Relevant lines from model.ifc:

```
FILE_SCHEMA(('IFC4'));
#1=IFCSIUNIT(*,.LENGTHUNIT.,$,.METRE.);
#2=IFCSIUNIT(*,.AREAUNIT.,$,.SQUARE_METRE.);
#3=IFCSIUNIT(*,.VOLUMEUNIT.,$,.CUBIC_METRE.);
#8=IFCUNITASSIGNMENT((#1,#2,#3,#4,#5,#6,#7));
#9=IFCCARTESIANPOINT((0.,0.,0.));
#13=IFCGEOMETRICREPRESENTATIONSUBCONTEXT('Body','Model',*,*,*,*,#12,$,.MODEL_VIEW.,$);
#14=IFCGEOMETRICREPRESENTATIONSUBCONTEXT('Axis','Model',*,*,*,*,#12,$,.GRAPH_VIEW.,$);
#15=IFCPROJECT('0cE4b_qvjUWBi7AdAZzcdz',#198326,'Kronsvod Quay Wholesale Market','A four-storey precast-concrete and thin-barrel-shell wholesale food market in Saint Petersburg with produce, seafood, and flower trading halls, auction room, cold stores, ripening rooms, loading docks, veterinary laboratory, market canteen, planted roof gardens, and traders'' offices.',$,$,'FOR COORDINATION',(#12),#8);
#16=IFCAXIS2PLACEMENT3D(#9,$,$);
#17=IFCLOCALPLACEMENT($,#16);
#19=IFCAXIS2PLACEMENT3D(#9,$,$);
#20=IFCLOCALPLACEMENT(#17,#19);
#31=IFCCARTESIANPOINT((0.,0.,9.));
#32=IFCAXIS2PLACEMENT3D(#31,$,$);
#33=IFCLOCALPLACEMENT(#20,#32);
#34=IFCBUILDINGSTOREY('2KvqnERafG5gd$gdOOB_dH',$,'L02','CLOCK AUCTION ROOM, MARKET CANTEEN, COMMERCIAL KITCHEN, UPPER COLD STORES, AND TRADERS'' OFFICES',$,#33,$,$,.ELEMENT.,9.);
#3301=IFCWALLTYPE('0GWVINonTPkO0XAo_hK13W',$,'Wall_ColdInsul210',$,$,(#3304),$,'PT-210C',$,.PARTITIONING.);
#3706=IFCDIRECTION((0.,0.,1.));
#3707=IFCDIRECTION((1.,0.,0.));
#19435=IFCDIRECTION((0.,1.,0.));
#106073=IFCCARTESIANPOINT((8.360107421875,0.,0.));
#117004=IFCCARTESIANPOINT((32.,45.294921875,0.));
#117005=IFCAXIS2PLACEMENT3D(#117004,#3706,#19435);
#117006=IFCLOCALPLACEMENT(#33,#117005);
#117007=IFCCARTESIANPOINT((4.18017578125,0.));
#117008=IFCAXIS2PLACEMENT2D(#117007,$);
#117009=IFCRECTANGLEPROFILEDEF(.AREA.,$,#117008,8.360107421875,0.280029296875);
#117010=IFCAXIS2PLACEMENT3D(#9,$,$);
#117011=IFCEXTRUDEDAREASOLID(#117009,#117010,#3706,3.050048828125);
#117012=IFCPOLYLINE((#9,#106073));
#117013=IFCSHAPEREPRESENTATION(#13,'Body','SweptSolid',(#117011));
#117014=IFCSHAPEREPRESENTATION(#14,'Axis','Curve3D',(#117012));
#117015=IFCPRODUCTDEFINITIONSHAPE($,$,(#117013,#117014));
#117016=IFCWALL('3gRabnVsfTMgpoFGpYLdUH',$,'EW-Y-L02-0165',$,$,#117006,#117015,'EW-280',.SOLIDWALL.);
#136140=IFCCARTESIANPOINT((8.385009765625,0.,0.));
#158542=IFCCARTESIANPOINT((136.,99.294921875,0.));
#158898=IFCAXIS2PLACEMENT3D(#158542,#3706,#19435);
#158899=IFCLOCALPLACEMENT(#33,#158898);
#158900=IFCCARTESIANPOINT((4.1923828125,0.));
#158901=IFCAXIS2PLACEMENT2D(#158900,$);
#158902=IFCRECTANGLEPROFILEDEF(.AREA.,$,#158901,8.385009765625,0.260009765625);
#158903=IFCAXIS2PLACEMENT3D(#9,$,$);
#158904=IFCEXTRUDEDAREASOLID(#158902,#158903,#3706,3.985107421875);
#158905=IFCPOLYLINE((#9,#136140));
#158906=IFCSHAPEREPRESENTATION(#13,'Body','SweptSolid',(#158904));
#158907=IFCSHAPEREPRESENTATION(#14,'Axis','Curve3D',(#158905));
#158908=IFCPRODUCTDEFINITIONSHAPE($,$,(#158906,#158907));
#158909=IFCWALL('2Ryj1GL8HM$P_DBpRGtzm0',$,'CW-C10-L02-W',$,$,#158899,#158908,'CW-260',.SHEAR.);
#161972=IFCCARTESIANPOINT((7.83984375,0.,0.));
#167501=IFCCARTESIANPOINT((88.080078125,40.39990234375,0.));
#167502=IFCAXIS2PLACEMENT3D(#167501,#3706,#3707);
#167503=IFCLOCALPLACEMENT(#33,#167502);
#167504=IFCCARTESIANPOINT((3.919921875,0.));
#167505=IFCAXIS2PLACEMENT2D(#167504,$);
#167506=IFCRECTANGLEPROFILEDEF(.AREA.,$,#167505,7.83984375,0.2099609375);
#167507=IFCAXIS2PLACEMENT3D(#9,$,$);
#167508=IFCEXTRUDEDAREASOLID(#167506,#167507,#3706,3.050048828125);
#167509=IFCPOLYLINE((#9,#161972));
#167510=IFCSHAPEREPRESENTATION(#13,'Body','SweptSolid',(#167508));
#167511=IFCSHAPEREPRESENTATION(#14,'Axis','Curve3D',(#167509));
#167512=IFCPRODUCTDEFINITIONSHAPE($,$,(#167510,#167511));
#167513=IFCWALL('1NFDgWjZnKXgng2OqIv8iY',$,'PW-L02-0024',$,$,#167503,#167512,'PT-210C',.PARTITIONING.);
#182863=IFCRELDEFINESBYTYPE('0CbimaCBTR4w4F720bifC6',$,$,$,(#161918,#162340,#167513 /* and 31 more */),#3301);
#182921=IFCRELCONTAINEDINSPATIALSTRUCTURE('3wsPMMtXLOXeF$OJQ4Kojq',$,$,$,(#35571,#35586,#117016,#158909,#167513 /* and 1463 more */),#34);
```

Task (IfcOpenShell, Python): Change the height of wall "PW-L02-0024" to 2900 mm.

```python
import ifcopenshell
import ifcopenshell.geom
import ifcopenshell.util.representation
import ifcopenshell.util.shape
import ifcopenshell.util.unit

model = ifcopenshell.open("model.ifc")
unit_scale = ifcopenshell.util.unit.calculate_unit_scale(model)
settings = ifcopenshell.geom.settings()


def volume(element):
    """Net volume in cubic metres, openings subtracted."""
    shape = ifcopenshell.geom.create_shape(settings, element)
    return ifcopenshell.util.shape.get_volume(shape.geometry)


wall = model.by_id(167513)
before = volume(wall)

body = ifcopenshell.util.representation.get_representation(wall, "Model", "Body")
solid = body.Items[0]
old_height = solid.Depth
solid.Depth = 2.9 / unit_scale
after = volume(wall)

print(f"height {old_height:g} -> {solid.Depth:g}, volume {before:.3f} -> {after:.3f} m3")

model.write("model_v2.ifc")
```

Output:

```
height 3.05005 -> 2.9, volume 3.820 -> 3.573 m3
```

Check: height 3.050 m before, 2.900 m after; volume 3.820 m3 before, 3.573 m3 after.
